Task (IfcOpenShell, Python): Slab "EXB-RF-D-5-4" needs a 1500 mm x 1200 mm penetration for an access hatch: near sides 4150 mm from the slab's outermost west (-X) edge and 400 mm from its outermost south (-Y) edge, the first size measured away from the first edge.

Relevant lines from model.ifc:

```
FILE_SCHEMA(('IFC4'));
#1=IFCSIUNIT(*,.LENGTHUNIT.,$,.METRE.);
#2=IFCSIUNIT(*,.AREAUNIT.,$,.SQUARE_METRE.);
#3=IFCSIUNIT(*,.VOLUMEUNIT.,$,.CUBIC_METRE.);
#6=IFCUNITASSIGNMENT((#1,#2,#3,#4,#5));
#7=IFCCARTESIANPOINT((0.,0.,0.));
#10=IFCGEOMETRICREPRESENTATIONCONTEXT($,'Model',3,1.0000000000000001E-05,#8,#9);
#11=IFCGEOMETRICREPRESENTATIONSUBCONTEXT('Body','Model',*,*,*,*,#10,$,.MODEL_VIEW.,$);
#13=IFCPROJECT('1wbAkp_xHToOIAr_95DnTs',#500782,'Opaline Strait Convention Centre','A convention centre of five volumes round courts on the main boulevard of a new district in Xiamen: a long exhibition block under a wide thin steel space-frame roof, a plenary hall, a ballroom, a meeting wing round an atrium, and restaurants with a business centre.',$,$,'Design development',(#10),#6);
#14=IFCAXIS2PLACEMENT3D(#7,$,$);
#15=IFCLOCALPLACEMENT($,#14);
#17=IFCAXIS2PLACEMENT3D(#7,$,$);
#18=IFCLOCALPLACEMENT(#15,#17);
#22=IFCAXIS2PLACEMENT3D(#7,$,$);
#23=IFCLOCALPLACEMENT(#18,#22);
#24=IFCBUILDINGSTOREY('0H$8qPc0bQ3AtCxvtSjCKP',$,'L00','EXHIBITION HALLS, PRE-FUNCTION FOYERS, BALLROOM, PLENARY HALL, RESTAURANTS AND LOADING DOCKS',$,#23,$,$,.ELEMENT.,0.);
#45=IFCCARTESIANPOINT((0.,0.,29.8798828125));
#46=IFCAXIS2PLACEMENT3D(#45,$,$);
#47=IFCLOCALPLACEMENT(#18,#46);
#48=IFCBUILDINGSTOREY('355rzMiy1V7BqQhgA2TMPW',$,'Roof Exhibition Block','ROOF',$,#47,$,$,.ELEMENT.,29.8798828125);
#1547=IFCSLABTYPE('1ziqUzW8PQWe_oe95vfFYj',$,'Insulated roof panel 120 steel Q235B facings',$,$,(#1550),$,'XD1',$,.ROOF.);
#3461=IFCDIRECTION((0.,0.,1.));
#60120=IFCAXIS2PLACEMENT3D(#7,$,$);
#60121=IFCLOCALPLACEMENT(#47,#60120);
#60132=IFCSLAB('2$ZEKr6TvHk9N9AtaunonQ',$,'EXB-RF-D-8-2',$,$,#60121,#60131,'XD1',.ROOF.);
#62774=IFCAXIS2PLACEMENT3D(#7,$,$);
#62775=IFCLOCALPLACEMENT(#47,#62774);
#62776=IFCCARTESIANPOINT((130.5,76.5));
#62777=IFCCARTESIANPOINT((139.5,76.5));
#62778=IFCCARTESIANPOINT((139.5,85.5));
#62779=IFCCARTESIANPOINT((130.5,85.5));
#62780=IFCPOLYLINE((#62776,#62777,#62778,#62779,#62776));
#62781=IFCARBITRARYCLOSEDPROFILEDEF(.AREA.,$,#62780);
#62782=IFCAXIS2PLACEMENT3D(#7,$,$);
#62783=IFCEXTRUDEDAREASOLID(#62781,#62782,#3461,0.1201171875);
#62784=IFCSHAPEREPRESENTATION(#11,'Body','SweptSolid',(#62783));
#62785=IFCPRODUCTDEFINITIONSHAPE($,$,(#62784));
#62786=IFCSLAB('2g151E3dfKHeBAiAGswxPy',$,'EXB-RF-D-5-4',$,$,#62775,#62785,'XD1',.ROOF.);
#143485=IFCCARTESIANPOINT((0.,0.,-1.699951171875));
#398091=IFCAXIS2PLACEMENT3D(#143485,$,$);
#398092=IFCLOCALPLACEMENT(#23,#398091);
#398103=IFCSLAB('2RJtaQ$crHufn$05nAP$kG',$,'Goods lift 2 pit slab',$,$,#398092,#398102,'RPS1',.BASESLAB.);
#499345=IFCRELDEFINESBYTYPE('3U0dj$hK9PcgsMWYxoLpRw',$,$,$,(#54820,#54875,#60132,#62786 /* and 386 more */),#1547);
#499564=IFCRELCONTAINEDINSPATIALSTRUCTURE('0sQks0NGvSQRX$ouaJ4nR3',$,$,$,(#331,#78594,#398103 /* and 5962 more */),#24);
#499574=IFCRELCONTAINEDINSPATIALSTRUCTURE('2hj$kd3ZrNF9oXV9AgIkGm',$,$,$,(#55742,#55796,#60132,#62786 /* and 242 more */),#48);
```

```python
import numpy as np
import ifcopenshell
import ifcopenshell.api.feature
import ifcopenshell.api.geometry
import ifcopenshell.api.root
import ifcopenshell.geom
import ifcopenshell.util.placement
import ifcopenshell.util.representation
import ifcopenshell.util.shape
import ifcopenshell.util.unit

model = ifcopenshell.open("model.ifc")
unit_scale = ifcopenshell.util.unit.calculate_unit_scale(model)
settings = ifcopenshell.geom.settings()


def volume(element):
    """Net volume in cubic metres, openings subtracted."""
    shape = ifcopenshell.geom.create_shape(settings, element)
    return ifcopenshell.util.shape.get_volume(shape.geometry)


slab = model.by_id(62786)
before = volume(slab)

# Extent in the slab's own axes, in metres. The edges named are its -X and -Y sides.
slab_shape = ifcopenshell.geom.create_shape(settings, slab)
vertices = ifcopenshell.util.shape.get_vertices(slab_shape.geometry)
x_min, y_min, bottom = vertices.min(axis=0)
top = vertices[:, 2].max()

opening = ifcopenshell.api.root.create_entity(model, ifc_class="IfcOpeningElement", name="Access hatch opening", predefined_type="OPENING")
context = ifcopenshell.util.representation.get_context(model, "Model", "Body", "MODEL_VIEW")
width, depth = 1.5, 1.2
outline = [(0.0, 0.0), (width, 0.0), (width, depth), (0.0, depth), (0.0, 0.0)]
# Overshoot both faces by 50 mm so the cut is clean.
shape = ifcopenshell.api.geometry.add_slab_representation(
    model, context=context, depth=top - bottom + 0.1, polyline=outline
)
ifcopenshell.api.geometry.assign_representation(model, product=opening, representation=shape)

matrix = ifcopenshell.util.placement.get_local_placement(slab.ObjectPlacement)
matrix[:, 3] = matrix @ np.append(np.array([x_min + 4.15, y_min + 0.4, bottom - 0.05]) / unit_scale, 1.0)
ifcopenshell.api.geometry.edit_object_placement(model, product=opening, matrix=matrix, is_si=False)
ifcopenshell.api.feature.add_feature(model, feature=opening, element=slab)

after = volume(slab)

print(f"slab volume {before:.3f} -> {after:.3f} m3")

model.write("model_updated.ifc")
```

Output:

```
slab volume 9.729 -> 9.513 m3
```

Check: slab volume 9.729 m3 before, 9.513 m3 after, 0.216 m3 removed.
